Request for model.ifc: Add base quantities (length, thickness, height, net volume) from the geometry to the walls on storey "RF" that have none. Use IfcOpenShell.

First a look at what the model holds.

```python
import ifcopenshell
import ifcopenshell.util.element
import ifcopenshell.util.unit

model = ifcopenshell.open("model.ifc")
print(model.schema)
for unit_type in ("LENGTHUNIT", "AREAUNIT", "VOLUMEUNIT"):
    print(unit_type, ifcopenshell.util.unit.calculate_unit_scale(model, unit_type))
storey = next(s for s in model.by_type("IfcBuildingStorey") if s.Name == "RF")
walls = [e for e in ifcopenshell.util.element.get_decomposition(storey) if e.is_a("IfcWall")]
for e in sorted(walls, key=lambda e: e.id()):
    print(e.id(), e.is_a(), e.Name, list(ifcopenshell.util.element.get_psets(e, qtos_only=True)), sep=" | ")
```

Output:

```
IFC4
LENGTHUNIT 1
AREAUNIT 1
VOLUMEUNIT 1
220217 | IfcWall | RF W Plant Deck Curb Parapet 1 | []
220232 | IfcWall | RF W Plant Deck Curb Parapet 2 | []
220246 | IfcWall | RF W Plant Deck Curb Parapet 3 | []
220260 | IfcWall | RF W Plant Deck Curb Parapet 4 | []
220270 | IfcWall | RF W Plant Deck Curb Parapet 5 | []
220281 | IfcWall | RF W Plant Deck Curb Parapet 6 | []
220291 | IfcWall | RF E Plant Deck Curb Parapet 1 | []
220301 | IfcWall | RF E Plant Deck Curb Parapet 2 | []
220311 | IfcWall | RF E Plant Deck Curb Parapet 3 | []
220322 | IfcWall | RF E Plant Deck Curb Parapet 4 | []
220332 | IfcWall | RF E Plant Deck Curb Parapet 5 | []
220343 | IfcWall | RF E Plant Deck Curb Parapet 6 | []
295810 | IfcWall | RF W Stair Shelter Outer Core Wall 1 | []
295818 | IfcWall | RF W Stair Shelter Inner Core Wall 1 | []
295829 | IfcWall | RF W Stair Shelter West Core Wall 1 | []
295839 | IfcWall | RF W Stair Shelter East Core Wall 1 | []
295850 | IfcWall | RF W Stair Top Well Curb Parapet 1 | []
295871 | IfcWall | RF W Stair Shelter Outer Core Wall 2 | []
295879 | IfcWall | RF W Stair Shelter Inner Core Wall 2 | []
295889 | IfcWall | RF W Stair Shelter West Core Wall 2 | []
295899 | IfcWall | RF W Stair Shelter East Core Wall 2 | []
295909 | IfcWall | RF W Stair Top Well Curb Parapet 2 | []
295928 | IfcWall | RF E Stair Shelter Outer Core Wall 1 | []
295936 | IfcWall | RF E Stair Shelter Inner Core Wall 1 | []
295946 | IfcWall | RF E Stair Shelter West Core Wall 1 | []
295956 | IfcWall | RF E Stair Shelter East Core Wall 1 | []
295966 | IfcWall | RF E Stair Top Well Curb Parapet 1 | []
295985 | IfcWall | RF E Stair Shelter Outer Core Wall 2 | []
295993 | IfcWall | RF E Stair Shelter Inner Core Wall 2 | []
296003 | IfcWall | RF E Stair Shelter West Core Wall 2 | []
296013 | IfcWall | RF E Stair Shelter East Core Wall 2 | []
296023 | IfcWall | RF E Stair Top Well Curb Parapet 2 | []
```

```python
import ifcopenshell
import ifcopenshell.api.pset
import ifcopenshell.geom
import ifcopenshell.util.element
import ifcopenshell.util.shape
import ifcopenshell.util.unit

model = ifcopenshell.open("model.ifc")
unit_scale = ifcopenshell.util.unit.calculate_unit_scale(model)
volume_scale = ifcopenshell.util.unit.calculate_unit_scale(model, "VOLUMEUNIT")
settings = ifcopenshell.geom.settings()

storey = next(s for s in model.by_type("IfcBuildingStorey") if s.Name == "RF")
walls = [e for e in ifcopenshell.util.element.get_decomposition(storey) if e.is_a("IfcWall")]

for e in sorted(walls, key=lambda e: e.id()):
    if ifcopenshell.util.element.get_psets(e, qtos_only=True, should_inherit=False):
        continue
    # Geometry comes back in metres, in the element's own axes.
    shape = ifcopenshell.geom.create_shape(settings, e)
    values = {
        "Length": ifcopenshell.util.shape.get_x(shape.geometry) / unit_scale,
        "Width": ifcopenshell.util.shape.get_y(shape.geometry) / unit_scale,
        "Height": ifcopenshell.util.shape.get_z(shape.geometry) / unit_scale,
        "NetVolume": ifcopenshell.util.shape.get_volume(shape.geometry) / volume_scale,
    }
    qto = ifcopenshell.api.pset.add_qto(model, product=e, name="Qto_WallBaseQuantities")
    ifcopenshell.api.pset.edit_qto(model, qto=qto, properties=values)
    print(e.id(), {k: round(v, 3) for k, v in values.items()})

model.write("model_edited.ifc")
```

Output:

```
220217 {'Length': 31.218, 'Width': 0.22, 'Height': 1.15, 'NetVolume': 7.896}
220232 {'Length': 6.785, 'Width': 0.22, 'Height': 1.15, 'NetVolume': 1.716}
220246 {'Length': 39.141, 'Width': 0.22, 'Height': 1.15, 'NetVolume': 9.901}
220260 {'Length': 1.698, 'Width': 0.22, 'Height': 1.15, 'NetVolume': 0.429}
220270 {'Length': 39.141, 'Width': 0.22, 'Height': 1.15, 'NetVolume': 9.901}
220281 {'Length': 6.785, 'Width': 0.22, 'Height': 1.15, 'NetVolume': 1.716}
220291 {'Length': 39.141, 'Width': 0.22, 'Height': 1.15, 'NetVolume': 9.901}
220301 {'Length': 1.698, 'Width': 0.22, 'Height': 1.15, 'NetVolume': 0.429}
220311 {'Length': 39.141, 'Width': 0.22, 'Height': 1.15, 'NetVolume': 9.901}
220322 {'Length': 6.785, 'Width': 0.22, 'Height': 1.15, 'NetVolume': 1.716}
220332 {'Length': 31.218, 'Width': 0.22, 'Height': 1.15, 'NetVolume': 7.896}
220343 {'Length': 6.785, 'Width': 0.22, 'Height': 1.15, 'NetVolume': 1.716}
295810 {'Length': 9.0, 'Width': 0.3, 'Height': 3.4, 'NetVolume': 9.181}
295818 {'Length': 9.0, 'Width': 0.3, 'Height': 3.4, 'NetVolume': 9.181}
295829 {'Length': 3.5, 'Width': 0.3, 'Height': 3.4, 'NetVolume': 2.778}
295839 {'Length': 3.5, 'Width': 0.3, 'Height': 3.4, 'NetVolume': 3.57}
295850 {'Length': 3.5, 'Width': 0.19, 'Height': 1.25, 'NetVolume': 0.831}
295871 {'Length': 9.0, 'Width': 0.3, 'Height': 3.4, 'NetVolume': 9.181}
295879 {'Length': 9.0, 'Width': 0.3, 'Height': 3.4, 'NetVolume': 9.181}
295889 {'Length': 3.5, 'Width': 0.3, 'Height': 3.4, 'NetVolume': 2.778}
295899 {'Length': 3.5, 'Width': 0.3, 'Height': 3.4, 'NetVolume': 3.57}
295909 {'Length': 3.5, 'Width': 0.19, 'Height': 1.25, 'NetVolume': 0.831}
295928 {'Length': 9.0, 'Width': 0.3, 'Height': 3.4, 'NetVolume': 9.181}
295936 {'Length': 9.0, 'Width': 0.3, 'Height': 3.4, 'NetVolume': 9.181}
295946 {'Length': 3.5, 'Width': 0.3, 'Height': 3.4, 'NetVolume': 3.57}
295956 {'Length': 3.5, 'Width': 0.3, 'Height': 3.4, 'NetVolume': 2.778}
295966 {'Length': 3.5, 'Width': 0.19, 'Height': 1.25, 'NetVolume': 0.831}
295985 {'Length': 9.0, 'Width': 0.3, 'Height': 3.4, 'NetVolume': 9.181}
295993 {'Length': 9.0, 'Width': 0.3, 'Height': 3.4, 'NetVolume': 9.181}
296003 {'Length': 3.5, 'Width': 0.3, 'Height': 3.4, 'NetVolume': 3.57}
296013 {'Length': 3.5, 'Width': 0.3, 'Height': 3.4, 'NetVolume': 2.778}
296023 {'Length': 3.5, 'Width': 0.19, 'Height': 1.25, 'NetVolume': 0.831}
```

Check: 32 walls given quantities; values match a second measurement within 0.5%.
